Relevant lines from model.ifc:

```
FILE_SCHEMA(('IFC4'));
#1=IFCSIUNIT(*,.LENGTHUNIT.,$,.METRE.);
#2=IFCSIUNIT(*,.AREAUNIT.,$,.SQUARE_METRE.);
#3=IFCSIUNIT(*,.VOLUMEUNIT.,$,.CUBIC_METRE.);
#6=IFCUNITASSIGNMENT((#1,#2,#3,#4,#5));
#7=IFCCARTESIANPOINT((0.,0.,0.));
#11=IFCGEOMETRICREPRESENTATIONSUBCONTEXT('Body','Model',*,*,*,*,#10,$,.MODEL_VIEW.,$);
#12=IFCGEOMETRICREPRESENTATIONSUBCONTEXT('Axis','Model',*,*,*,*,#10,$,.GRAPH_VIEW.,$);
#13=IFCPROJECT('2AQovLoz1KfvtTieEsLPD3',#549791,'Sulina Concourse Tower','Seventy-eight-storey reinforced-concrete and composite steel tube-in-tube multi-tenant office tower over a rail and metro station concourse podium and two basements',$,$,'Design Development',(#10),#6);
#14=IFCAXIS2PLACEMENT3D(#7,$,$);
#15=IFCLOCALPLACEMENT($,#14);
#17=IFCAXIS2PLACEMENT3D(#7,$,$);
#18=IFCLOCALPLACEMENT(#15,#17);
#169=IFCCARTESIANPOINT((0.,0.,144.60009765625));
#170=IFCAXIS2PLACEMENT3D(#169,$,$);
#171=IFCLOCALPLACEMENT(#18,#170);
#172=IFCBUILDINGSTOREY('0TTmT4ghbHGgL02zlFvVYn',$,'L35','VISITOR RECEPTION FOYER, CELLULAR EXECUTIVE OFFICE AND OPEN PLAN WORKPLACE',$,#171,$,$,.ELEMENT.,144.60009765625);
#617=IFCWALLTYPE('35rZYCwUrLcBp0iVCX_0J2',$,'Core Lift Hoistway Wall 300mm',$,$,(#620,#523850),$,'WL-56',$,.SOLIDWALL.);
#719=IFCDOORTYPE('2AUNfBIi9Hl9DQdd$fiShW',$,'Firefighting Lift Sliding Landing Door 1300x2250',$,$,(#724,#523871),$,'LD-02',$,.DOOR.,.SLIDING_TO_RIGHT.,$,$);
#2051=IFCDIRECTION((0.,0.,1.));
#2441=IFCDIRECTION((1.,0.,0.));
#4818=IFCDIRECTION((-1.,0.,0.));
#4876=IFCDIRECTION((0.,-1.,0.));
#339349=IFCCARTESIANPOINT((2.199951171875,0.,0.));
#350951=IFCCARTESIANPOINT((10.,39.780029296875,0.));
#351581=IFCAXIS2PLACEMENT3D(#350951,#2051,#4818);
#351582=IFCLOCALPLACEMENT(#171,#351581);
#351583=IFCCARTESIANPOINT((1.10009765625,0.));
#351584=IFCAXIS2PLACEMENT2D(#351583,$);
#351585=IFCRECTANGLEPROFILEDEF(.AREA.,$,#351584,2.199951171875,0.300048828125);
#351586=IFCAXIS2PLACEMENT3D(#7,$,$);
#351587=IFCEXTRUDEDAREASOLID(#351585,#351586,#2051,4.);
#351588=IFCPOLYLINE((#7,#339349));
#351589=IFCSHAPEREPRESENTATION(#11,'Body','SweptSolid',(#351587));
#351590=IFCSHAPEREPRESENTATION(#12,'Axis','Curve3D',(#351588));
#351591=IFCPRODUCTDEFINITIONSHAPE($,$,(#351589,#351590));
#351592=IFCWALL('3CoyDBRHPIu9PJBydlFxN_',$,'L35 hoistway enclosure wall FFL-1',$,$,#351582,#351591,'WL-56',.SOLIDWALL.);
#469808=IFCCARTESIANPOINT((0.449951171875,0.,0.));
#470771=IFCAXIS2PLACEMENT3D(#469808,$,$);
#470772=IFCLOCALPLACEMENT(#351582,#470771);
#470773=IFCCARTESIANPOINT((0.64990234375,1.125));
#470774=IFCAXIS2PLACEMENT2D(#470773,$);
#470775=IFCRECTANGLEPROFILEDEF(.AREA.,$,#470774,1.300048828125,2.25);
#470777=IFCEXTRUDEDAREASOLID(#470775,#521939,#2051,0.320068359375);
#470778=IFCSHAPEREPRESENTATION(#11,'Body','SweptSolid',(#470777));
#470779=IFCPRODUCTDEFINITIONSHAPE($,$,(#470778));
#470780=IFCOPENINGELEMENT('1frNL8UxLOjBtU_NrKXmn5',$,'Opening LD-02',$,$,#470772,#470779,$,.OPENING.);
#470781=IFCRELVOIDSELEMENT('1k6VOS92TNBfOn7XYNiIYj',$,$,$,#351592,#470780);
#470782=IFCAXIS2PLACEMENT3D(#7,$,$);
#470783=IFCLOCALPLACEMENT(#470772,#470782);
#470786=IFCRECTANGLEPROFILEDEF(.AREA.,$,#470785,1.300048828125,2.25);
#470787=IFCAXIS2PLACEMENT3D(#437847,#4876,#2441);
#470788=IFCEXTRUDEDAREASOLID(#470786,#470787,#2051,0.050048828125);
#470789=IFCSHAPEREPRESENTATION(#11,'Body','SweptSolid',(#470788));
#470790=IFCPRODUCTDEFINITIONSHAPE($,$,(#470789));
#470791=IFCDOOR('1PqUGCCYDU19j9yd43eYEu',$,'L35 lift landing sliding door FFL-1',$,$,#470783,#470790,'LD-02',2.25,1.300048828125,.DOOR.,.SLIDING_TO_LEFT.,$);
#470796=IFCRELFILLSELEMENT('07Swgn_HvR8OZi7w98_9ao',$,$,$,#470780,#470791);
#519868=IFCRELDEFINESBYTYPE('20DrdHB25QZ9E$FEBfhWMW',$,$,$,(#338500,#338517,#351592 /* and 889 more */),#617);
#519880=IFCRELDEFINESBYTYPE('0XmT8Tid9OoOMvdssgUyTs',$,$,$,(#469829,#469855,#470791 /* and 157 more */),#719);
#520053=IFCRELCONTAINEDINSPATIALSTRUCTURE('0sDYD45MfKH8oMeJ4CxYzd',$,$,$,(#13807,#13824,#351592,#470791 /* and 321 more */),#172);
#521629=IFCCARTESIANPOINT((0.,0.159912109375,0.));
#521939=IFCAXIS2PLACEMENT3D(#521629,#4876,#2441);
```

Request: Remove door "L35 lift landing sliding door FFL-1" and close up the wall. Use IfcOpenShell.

```python
import ifcopenshell
import ifcopenshell.api.feature
import ifcopenshell.api.root
import ifcopenshell.geom
import ifcopenshell.util.shape

model = ifcopenshell.open("model.ifc")
settings = ifcopenshell.geom.settings()


def volume(element):
    """Net volume in cubic metres, openings subtracted."""
    shape = ifcopenshell.geom.create_shape(settings, element)
    return ifcopenshell.util.shape.get_volume(shape.geometry)


door = model.by_guid("1PqUGCCYDU19j9yd43eYEu")
opening = door.FillsVoids[0].RelatingOpeningElement
wall = opening.VoidsElements[0].RelatingBuildingElement
before = volume(wall)

ifcopenshell.api.root.remove_product(model, product=door)
ifcopenshell.api.feature.remove_feature(model, feature=opening)

after = volume(wall)

print(f"wall volume {before:.3f} -> {after:.3f} m3")

model.write("model_rev.ifc")
```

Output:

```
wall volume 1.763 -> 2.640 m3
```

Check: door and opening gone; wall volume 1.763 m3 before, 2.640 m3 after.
